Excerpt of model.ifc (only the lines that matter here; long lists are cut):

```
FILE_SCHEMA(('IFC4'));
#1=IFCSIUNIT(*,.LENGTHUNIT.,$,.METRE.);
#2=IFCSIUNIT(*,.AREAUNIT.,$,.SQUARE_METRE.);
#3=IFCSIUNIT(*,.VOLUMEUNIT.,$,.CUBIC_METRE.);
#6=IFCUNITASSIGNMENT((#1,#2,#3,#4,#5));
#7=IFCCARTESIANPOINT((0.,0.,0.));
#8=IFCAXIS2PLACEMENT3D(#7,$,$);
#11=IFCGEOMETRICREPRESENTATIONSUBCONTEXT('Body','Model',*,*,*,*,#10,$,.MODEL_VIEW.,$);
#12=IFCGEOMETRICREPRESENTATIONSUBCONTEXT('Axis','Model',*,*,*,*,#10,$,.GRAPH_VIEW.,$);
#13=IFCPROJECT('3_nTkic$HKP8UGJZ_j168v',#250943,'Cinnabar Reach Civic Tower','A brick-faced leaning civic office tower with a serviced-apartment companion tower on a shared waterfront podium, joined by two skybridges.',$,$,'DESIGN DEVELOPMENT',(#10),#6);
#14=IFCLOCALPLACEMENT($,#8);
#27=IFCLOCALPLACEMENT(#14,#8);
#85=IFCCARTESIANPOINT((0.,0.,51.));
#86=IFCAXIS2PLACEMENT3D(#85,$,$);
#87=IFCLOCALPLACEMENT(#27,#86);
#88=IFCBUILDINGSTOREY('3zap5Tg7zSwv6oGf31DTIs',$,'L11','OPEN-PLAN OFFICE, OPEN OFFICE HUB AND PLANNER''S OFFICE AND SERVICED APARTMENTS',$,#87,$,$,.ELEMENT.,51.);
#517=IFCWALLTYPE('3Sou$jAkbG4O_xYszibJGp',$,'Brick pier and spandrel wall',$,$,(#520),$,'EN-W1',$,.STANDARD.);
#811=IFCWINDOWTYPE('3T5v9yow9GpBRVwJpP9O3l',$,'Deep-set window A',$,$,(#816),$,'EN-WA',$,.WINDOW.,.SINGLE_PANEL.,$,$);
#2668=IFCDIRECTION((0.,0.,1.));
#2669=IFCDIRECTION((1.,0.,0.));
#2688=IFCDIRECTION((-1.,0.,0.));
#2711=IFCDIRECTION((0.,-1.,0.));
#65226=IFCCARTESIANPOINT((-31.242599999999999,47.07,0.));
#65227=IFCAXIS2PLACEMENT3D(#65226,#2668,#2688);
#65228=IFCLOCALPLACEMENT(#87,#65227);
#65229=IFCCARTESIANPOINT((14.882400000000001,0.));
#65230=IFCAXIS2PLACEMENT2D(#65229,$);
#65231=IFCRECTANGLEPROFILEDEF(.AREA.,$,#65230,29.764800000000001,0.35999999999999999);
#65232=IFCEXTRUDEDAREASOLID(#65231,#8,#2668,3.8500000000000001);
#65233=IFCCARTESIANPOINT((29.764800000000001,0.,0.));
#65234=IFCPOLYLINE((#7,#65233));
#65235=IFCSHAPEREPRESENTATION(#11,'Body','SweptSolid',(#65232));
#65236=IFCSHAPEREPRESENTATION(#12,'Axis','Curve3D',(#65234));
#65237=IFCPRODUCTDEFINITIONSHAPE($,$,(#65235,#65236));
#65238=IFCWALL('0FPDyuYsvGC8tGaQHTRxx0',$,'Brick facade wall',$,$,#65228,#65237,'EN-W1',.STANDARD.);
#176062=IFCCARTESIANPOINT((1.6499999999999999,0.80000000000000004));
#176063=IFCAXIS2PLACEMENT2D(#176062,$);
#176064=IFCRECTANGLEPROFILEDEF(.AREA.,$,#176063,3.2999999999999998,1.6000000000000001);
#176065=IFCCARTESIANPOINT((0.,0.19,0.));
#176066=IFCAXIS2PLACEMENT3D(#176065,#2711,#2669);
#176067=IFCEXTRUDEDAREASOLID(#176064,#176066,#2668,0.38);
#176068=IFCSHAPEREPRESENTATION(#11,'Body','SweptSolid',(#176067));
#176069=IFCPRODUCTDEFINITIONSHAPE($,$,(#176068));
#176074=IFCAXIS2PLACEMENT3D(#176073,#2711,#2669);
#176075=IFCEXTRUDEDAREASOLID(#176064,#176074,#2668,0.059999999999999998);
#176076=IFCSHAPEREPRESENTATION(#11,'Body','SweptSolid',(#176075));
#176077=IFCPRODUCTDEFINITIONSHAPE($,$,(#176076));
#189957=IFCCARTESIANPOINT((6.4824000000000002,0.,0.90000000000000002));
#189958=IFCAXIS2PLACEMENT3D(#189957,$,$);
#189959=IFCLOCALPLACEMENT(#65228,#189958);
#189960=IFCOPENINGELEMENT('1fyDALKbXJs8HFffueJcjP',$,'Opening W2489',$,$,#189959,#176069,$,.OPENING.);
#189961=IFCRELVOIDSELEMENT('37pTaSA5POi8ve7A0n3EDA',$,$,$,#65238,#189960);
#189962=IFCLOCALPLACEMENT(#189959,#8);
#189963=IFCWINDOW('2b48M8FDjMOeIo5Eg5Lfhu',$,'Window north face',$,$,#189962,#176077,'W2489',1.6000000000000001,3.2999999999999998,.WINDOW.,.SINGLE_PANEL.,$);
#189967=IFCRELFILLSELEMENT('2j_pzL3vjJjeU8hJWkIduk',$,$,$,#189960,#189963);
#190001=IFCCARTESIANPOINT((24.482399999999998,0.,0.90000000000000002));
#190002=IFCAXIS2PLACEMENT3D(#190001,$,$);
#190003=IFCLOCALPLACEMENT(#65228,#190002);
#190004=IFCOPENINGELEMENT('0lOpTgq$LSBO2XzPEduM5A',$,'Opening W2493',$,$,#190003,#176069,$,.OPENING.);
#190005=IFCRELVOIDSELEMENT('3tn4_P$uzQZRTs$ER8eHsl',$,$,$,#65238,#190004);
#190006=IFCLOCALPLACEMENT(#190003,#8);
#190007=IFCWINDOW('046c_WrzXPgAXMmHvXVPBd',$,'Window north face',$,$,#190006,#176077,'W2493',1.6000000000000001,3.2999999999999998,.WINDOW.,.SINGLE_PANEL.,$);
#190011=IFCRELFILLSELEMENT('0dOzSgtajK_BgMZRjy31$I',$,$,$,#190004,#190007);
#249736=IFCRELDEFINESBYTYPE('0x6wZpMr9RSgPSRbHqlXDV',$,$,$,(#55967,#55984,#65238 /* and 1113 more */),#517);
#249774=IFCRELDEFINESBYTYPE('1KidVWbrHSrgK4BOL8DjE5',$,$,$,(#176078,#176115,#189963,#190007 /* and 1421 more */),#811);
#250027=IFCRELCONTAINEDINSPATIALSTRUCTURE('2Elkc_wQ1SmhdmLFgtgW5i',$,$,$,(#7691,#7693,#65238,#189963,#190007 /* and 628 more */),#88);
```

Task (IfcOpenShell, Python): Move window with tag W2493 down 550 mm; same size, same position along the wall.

```python
import numpy as np
import ifcopenshell
import ifcopenshell.api.geometry
import ifcopenshell.util.placement
import ifcopenshell.util.unit

model = ifcopenshell.open("model.ifc")
unit_scale = ifcopenshell.util.unit.calculate_unit_scale(model)

window = model.by_guid("046c_WrzXPgAXMmHvXVPBd")
opening = window.FillsVoids[0].RelatingOpeningElement
dz = -0.55 / unit_scale

shift = np.array([0.0, 0.0, dz])
# The window is placed relative to its opening, so it follows when the opening moves.
matrix = ifcopenshell.util.placement.get_local_placement(opening.ObjectPlacement)
matrix[:3, 3] += shift
ifcopenshell.api.geometry.edit_object_placement(
    model, product=opening, matrix=matrix, is_si=False, should_transform_children=True
)

print(f"moved by {dz * unit_scale:+.3f} m")

model.write("model_updated.ifc")
```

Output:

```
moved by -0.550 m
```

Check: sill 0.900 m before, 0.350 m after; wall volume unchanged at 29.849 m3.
